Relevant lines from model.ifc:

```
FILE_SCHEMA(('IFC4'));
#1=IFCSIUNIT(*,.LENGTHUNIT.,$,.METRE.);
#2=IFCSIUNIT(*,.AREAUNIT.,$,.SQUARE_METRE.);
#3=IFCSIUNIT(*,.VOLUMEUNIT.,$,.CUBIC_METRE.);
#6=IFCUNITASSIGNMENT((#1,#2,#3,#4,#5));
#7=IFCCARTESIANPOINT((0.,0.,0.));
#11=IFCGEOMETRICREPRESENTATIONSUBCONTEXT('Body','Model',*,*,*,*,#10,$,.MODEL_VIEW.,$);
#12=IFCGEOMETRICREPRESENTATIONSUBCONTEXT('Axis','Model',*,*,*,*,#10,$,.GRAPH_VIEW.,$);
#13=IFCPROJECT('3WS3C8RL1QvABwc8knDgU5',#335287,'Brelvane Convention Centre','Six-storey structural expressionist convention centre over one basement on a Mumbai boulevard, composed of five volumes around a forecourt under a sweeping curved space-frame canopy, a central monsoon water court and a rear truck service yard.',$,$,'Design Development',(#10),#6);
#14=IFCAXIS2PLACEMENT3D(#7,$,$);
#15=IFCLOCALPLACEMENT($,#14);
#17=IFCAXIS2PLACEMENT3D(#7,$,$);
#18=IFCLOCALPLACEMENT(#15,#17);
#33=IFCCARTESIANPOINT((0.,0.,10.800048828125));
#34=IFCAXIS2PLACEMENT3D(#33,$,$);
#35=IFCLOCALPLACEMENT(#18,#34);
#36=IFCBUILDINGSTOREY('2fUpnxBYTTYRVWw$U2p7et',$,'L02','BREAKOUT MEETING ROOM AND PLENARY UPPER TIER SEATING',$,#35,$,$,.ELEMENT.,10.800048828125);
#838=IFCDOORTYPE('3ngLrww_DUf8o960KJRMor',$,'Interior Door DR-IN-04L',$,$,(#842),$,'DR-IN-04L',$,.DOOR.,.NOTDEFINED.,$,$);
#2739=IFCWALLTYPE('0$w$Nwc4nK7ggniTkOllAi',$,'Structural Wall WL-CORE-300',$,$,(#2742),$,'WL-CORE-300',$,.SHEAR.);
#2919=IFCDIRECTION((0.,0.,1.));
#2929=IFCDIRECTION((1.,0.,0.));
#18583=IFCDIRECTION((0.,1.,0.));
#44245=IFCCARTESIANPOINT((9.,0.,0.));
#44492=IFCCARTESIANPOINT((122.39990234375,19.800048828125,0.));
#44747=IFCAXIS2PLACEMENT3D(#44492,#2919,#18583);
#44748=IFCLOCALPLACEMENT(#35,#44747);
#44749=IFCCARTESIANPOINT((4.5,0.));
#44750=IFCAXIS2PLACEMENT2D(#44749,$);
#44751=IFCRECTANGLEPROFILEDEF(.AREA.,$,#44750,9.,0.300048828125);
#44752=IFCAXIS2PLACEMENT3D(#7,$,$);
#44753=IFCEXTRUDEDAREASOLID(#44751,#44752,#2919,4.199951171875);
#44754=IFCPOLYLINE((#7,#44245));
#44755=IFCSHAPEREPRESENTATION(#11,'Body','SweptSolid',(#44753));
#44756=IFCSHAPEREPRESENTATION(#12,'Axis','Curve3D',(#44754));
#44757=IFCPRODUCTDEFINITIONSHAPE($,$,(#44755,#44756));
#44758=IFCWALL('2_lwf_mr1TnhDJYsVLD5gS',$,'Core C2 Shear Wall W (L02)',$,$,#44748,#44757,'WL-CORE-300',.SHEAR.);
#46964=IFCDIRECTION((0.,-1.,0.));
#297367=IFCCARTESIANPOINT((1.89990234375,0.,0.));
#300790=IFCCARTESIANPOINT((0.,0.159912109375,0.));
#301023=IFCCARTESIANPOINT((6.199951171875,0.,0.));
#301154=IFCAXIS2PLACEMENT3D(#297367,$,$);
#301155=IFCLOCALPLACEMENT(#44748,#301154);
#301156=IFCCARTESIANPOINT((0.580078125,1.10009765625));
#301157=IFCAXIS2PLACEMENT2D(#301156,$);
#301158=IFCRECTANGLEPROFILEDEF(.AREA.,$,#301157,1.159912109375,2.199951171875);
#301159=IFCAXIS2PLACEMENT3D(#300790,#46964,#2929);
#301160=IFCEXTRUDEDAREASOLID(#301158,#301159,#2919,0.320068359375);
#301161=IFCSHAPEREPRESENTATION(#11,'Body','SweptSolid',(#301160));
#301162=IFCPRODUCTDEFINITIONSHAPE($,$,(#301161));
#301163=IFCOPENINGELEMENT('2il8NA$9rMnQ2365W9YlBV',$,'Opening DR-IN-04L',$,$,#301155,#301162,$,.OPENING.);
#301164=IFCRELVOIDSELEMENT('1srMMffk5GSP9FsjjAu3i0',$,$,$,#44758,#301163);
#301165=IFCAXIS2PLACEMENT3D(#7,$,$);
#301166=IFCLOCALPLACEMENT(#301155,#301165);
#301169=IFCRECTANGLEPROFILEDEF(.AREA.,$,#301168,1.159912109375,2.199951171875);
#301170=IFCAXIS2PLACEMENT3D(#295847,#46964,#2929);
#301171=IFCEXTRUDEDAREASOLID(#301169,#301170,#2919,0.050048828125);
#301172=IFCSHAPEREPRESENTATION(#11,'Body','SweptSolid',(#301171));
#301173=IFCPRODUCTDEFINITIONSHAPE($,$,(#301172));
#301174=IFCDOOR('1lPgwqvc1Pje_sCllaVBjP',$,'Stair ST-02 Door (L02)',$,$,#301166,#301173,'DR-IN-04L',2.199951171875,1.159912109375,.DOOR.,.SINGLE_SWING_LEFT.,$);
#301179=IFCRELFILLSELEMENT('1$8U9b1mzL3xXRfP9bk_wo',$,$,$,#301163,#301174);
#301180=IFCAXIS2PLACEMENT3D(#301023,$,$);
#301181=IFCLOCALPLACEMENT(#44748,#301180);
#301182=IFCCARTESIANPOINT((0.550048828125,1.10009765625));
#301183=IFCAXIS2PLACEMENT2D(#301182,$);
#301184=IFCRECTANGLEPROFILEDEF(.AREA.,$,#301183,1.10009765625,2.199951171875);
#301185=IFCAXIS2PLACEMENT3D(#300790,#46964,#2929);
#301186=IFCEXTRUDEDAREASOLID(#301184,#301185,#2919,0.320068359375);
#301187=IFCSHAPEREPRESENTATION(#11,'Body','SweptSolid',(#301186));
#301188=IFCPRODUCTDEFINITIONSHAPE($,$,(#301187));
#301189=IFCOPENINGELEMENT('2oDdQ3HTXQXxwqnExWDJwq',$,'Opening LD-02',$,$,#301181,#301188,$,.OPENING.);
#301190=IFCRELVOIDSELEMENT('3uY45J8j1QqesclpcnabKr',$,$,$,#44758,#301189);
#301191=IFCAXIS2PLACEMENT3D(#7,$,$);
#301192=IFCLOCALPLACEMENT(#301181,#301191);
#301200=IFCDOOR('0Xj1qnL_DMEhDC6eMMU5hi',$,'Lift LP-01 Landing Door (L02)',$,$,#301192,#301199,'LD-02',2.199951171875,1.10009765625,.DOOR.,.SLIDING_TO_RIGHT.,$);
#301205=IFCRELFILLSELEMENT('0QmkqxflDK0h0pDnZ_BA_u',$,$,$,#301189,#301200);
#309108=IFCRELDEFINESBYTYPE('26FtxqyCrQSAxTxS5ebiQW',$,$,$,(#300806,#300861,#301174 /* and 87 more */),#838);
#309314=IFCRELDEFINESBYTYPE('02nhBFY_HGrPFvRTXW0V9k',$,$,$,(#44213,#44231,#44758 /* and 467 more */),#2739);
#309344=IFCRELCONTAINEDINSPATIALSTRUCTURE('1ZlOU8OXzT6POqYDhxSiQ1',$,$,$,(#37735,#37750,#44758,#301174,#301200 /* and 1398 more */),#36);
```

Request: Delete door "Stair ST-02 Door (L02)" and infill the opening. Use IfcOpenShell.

```python
import ifcopenshell
import ifcopenshell.api.feature
import ifcopenshell.api.root
import ifcopenshell.geom
import ifcopenshell.util.shape

model = ifcopenshell.open("model.ifc")
settings = ifcopenshell.geom.settings()


def volume(element):
    """Net volume in cubic metres, openings subtracted."""
    shape = ifcopenshell.geom.create_shape(settings, element)
    return ifcopenshell.util.shape.get_volume(shape.geometry)


door = model.by_id(301174)
opening = door.FillsVoids[0].RelatingOpeningElement
wall = opening.VoidsElements[0].RelatingBuildingElement
before = volume(wall)

ifcopenshell.api.root.remove_product(model, product=door)
ifcopenshell.api.feature.remove_feature(model, feature=opening)

after = volume(wall)

print(f"wall volume {before:.3f} -> {after:.3f} m3")

model.write("model_rev.ifc")
```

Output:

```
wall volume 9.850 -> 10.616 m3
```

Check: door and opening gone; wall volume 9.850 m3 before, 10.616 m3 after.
